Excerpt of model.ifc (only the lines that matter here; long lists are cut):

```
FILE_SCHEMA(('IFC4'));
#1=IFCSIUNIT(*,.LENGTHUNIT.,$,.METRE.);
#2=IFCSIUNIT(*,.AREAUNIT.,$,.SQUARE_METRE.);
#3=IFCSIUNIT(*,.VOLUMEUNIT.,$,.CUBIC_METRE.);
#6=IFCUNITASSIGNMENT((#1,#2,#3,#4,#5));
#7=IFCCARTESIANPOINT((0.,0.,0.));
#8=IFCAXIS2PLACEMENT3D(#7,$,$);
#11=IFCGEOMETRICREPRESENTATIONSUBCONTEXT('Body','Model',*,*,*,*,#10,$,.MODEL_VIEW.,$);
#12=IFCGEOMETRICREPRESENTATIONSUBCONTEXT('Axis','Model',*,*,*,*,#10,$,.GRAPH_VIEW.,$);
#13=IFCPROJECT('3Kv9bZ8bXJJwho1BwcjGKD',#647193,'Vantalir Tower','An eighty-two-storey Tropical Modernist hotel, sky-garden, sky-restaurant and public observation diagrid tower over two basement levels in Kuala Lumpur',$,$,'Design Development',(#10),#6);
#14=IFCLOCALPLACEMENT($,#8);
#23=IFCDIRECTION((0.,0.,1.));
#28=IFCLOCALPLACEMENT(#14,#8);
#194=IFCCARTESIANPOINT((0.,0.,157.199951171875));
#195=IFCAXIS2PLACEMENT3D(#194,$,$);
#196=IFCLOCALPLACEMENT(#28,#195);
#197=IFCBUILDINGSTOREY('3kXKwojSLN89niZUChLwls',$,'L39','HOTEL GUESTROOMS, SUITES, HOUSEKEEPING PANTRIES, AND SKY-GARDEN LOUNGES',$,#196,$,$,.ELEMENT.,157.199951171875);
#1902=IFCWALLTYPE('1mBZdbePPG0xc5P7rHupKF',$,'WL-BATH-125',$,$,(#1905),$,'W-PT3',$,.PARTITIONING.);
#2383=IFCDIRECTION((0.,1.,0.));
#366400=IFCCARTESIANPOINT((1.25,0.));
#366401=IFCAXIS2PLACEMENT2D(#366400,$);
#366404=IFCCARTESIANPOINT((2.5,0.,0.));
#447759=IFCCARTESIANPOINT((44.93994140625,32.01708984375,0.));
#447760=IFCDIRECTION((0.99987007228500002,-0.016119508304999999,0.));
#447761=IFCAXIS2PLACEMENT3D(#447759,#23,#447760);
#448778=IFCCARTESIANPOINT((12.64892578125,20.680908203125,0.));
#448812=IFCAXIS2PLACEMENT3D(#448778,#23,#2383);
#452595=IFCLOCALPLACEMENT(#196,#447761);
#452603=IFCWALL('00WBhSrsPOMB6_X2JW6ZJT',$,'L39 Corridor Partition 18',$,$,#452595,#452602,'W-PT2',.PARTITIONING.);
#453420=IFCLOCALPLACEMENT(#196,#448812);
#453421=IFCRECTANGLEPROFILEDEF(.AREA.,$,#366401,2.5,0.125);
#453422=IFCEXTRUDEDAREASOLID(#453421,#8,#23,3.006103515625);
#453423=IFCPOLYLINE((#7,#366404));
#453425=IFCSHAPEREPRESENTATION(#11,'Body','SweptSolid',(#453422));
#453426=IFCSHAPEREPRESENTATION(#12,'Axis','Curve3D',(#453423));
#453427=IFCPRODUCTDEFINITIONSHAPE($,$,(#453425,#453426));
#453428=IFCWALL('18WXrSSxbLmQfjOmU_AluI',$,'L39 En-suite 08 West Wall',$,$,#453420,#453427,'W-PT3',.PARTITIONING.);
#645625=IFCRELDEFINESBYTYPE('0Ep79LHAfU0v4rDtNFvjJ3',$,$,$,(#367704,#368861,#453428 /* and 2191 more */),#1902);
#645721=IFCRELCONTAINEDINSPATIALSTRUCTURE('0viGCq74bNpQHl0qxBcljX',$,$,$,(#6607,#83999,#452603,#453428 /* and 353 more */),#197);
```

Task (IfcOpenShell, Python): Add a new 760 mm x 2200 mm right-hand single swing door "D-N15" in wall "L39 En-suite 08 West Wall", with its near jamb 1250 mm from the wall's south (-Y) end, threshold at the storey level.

```python
import numpy as np
import ifcopenshell
import ifcopenshell.api.feature
import ifcopenshell.api.geometry
import ifcopenshell.api.root
import ifcopenshell.api.spatial
import ifcopenshell.geom
import ifcopenshell.util.element
import ifcopenshell.util.placement
import ifcopenshell.util.representation
import ifcopenshell.util.shape
import ifcopenshell.util.unit

model = ifcopenshell.open("model.ifc")
unit_scale = ifcopenshell.util.unit.calculate_unit_scale(model)
settings = ifcopenshell.geom.settings()


def volume(element):
    """Net volume in cubic metres, openings subtracted."""
    shape = ifcopenshell.geom.create_shape(settings, element)
    return ifcopenshell.util.shape.get_volume(shape.geometry)


wall = model.by_guid("18WXrSSxbLmQfjOmU_AluI")
storey = ifcopenshell.util.element.get_container(wall, ifc_class="IfcBuildingStorey")
context = ifcopenshell.util.representation.get_context(model, "Model", "Body", "MODEL_VIEW")
before = volume(wall)

width, height, from_end, sill = 0.76, 2.2, 1.25, 0.0  # metres

# The wall runs along its own X axis, and the end named is its -X end.
wall_shape = ifcopenshell.geom.create_shape(settings, wall)
x, y, z = ifcopenshell.util.shape.get_vertices(wall_shape.geometry).T
start = x.min() + from_end
face, thickness = float(y.min()), float(y.max() - y.min())
wall_matrix = ifcopenshell.util.placement.get_local_placement(wall.ObjectPlacement)
level = ifcopenshell.util.placement.get_local_placement(storey.ObjectPlacement)[2, 3]


def in_wall(x, y):
    """Placement at x, y metres in the wall's axes, at sill height."""
    matrix = wall_matrix.copy()
    matrix[:, 3] = wall_matrix @ np.array([x / unit_scale, y / unit_scale, 0.0, 1.0])
    matrix[2, 3] = level + sill / unit_scale
    return matrix


# Opening: a box that overshoots both wall faces by 50 mm.
opening = ifcopenshell.api.root.create_entity(model, ifc_class="IfcOpeningElement", predefined_type="OPENING")
box = ifcopenshell.api.geometry.add_wall_representation(
    model, context=context, length=width, height=height, thickness=thickness + 0.1
)
ifcopenshell.api.geometry.assign_representation(model, product=opening, representation=box)
ifcopenshell.api.geometry.edit_object_placement(model, product=opening, matrix=in_wall(start, face - 0.05), is_si=False)
ifcopenshell.api.feature.add_feature(model, feature=opening, element=wall)

door = ifcopenshell.api.root.create_entity(model, ifc_class="IfcDoor", name="D-N15", predefined_type="DOOR")
door.OverallWidth, door.OverallHeight = width / unit_scale, height / unit_scale
door.OperationType = "SINGLE_SWING_RIGHT"
body = ifcopenshell.api.geometry.add_door_representation(
    model,
    context=context,
    overall_width=door.OverallWidth,
    overall_height=door.OverallHeight,
    operation_type="SINGLE_SWING_RIGHT",
    lining_properties={"LiningDepth": thickness / unit_scale, "ThresholdDepth": thickness / unit_scale},
)
ifcopenshell.api.geometry.assign_representation(model, product=door, representation=body)
ifcopenshell.api.spatial.assign_container(model, products=[door], relating_structure=storey)
ifcopenshell.api.feature.add_filling(model, opening=opening, element=door)

# The lining spans the wall, so the door starts at the wall face.
ifcopenshell.api.geometry.edit_object_placement(model, product=door, matrix=in_wall(start, face), is_si=False)

after = volume(wall)

print(f"wall volume {before:.3f} -> {after:.3f} m3")

model.write("model-out.ifc")
```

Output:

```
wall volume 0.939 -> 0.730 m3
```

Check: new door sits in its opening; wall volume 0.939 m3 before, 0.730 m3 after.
